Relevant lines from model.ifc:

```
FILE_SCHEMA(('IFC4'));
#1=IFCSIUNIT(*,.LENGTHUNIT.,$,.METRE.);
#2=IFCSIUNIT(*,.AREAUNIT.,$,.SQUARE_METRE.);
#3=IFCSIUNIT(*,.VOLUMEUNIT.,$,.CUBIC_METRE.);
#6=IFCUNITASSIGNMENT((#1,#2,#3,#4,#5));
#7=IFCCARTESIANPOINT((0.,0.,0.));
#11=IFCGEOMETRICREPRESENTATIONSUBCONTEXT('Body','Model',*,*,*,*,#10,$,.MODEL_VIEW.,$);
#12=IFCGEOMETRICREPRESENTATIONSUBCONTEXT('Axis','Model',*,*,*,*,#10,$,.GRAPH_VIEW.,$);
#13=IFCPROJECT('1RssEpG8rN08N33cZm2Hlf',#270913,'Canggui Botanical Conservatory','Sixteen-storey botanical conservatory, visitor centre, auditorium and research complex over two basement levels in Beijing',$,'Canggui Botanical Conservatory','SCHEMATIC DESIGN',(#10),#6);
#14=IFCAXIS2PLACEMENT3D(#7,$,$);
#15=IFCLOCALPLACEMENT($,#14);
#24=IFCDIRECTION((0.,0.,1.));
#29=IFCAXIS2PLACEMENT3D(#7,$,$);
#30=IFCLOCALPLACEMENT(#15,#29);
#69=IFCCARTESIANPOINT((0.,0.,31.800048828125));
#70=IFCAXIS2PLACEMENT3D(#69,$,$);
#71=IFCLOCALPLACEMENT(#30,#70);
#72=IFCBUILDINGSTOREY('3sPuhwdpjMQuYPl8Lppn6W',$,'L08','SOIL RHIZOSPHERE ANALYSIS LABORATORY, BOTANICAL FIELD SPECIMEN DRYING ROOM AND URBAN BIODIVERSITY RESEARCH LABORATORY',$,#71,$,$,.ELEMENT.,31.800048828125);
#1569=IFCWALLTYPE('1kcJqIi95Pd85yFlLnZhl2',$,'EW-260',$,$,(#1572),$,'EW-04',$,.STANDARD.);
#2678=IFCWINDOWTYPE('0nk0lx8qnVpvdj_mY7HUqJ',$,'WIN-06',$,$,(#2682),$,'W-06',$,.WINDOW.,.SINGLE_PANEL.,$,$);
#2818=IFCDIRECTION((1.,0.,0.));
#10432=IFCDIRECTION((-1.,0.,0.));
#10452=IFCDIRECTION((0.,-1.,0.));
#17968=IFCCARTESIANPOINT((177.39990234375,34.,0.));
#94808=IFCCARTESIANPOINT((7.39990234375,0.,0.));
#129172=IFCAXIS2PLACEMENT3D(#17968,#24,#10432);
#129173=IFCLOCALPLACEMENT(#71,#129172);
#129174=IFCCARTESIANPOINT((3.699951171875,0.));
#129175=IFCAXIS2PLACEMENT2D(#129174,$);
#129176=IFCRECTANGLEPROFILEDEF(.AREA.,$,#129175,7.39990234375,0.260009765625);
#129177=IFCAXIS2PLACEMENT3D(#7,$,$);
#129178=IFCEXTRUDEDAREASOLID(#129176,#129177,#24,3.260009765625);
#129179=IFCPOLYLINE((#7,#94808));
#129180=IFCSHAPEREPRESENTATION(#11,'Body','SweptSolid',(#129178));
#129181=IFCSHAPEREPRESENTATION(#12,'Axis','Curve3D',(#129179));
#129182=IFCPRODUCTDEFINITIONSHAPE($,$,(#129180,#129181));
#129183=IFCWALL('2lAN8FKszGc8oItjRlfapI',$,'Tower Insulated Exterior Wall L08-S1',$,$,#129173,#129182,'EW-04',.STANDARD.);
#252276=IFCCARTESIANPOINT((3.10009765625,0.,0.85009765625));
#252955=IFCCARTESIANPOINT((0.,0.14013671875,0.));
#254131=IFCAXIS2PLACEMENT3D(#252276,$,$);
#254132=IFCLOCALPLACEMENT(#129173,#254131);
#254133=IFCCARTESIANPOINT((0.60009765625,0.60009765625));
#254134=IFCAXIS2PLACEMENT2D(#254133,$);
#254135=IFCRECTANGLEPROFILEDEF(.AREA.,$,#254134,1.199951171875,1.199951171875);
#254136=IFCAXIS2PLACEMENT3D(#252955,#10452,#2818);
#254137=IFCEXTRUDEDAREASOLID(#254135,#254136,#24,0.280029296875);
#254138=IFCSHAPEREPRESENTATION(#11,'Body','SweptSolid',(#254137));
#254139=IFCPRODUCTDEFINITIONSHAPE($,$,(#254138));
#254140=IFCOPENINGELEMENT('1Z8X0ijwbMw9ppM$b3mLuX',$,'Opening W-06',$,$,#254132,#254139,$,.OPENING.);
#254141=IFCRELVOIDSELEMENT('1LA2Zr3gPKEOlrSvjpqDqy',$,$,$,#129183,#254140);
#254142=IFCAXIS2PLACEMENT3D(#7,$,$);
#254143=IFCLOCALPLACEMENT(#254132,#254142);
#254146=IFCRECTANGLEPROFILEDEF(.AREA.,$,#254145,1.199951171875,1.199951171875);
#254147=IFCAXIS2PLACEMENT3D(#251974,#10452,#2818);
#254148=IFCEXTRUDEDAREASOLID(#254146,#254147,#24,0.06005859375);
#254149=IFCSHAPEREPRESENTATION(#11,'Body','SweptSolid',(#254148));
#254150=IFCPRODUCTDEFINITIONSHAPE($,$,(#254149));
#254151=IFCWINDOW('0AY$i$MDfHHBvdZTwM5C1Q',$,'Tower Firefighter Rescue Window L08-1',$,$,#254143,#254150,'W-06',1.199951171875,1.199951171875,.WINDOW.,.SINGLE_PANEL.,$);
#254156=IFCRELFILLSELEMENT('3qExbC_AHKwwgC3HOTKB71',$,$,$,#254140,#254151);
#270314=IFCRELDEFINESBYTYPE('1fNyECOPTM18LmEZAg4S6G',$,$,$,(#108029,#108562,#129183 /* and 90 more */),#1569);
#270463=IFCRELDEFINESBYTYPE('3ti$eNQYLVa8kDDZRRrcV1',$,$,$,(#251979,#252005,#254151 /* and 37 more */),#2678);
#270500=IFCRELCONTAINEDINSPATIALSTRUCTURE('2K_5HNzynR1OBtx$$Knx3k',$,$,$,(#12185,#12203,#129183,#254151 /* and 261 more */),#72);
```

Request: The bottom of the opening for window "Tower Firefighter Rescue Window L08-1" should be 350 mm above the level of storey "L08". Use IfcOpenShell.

```python
import numpy as np
import ifcopenshell
import ifcopenshell.api.geometry
import ifcopenshell.geom
import ifcopenshell.util.element
import ifcopenshell.util.placement
import ifcopenshell.util.shape
import ifcopenshell.util.unit

model = ifcopenshell.open("model.ifc")
unit_scale = ifcopenshell.util.unit.calculate_unit_scale(model)

window = model.by_guid("0AY$i$MDfHHBvdZTwM5C1Q")
opening = window.FillsVoids[0].RelatingOpeningElement
storey = ifcopenshell.util.element.get_container(window, ifc_class="IfcBuildingStorey")
level = ifcopenshell.util.placement.get_local_placement(storey.ObjectPlacement)[2, 3]

# The opening's origin need not be at the sill, so measure its lowest point.
shape = ifcopenshell.geom.create_shape(ifcopenshell.geom.settings(), opening)
bottom = ifcopenshell.util.shape.get_shape_bottom_elevation(shape, shape.geometry) / unit_scale
dz = level + 0.35 / unit_scale - bottom

shift = np.array([0.0, 0.0, dz])
# The window is placed relative to its opening, so it follows when the opening moves.
matrix = ifcopenshell.util.placement.get_local_placement(opening.ObjectPlacement)
matrix[:3, 3] += shift
ifcopenshell.api.geometry.edit_object_placement(
    model, product=opening, matrix=matrix, is_si=False, should_transform_children=True
)

print(f"moved by {dz * unit_scale:+.3f} m")

model.write("model-out.ifc")
```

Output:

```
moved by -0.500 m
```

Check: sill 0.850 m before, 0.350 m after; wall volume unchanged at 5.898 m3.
